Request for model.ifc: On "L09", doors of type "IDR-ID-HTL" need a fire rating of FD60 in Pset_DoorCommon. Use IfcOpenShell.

First a look at what the model holds.

```python
import ifcopenshell
import ifcopenshell.util.element

model = ifcopenshell.open("model.ifc")
print(model.schema)
storey = next(s for s in model.by_type("IfcBuildingStorey") if s.Name == "L09")
doors = [e for e in ifcopenshell.util.element.get_decomposition(storey) if e.is_a("IfcDoor")]
seen = {}
for e in doors:
    element_type = ifcopenshell.util.element.get_type(e)
    key = (element_type.Name if element_type != e and element_type else None, ifcopenshell.util.element.get_pset(e, "Pset_DoorCommon", "FireRating"))
    seen[key] = seen.get(key, 0) + 1
for (name, value), count in sorted(seen.items(), key=str):
    print(count, "x", name, "|", value)
```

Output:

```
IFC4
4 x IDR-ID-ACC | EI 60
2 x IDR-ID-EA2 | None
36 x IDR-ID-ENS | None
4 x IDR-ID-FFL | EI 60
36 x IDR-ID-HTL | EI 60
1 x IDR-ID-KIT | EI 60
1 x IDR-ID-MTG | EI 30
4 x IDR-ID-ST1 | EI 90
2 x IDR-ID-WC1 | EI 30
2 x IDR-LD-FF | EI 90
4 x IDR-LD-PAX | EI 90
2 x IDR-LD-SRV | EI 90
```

```python
import ifcopenshell
import ifcopenshell.api.pset
import ifcopenshell.util.element

model = ifcopenshell.open("model.ifc")

storey = next(s for s in model.by_type("IfcBuildingStorey") if s.Name == "L09")
doors = [e for e in ifcopenshell.util.element.get_decomposition(storey) if e.is_a("IfcDoor")]

count = 0
for e in doors:
    element_type = ifcopenshell.util.element.get_type(e)
    if element_type in (None, e) or element_type.Name != "IDR-ID-HTL":
        continue
    # add_pset returns the element's existing set when there is one.
    pset = ifcopenshell.api.pset.add_pset(model, product=e, name="Pset_DoorCommon")
    ifcopenshell.api.pset.edit_pset(model, pset=pset, properties={"FireRating": "FD60"})
    count += 1

print(count, "doors updated")

model.write("model_v2.ifc")
```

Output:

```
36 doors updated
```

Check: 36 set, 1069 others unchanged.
